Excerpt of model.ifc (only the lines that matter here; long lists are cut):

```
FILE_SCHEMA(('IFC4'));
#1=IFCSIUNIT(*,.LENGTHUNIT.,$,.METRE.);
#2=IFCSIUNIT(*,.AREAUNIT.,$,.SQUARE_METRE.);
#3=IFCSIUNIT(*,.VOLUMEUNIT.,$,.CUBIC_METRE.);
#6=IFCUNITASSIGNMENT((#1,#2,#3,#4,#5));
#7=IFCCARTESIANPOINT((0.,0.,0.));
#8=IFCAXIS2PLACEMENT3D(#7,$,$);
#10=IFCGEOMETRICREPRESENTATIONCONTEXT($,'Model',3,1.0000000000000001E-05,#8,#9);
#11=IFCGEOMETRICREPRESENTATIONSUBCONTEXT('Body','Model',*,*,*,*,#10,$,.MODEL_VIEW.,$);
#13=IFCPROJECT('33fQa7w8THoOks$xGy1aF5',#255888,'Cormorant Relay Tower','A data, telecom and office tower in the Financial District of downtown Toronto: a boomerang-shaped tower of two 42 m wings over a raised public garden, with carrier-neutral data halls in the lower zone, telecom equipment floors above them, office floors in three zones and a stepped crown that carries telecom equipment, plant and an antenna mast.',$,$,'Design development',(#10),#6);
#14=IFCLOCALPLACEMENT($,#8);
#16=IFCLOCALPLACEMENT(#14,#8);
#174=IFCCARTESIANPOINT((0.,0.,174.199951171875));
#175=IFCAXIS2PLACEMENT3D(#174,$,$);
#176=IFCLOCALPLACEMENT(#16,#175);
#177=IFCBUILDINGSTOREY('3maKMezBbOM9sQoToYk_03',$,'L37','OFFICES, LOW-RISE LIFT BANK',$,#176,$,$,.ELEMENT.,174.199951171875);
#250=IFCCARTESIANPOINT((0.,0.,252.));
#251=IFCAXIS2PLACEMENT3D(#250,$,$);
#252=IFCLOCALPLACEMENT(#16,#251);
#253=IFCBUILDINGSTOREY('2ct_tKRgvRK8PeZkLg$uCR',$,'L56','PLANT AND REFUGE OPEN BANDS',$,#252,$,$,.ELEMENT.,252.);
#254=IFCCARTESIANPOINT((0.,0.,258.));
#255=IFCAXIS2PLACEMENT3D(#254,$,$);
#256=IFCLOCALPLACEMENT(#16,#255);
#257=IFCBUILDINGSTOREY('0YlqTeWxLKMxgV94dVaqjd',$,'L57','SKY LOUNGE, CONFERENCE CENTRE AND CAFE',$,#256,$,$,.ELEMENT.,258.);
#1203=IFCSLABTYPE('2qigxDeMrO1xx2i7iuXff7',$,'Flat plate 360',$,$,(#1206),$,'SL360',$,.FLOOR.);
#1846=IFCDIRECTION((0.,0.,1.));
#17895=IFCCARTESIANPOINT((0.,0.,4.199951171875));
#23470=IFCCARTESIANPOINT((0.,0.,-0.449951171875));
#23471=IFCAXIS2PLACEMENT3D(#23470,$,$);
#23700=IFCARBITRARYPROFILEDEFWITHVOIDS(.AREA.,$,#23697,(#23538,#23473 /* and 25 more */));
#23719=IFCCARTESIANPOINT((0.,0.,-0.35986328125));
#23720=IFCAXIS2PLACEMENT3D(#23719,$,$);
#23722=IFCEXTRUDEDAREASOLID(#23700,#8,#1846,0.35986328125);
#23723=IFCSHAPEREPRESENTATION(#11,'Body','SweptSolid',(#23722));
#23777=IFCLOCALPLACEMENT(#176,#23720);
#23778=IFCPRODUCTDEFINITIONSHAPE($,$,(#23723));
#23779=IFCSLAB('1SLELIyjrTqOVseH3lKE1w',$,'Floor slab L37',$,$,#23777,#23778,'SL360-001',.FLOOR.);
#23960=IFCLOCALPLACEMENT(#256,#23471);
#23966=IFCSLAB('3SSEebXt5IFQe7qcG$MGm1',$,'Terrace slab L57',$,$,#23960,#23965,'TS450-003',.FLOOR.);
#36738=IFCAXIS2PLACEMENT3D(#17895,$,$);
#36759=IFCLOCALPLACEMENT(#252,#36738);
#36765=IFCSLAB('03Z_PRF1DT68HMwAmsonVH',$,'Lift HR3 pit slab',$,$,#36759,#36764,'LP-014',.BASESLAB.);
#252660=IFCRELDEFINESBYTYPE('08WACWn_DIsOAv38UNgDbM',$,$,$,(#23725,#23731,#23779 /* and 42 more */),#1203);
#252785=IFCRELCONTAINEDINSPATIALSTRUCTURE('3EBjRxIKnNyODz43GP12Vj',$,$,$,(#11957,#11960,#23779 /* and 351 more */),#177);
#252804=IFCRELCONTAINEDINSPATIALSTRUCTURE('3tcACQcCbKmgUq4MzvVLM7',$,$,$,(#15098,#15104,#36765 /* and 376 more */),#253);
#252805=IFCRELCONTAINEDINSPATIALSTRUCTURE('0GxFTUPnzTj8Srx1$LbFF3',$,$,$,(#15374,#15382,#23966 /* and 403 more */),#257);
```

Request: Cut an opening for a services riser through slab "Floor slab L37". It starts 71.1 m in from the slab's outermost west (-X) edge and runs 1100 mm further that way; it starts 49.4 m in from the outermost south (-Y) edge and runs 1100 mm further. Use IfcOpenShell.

```python
import numpy as np
import ifcopenshell
import ifcopenshell.api.feature
import ifcopenshell.api.geometry
import ifcopenshell.api.root
import ifcopenshell.geom
import ifcopenshell.util.placement
import ifcopenshell.util.representation
import ifcopenshell.util.shape
import ifcopenshell.util.unit

model = ifcopenshell.open("model.ifc")
unit_scale = ifcopenshell.util.unit.calculate_unit_scale(model)
settings = ifcopenshell.geom.settings()


def volume(element):
    """Net volume in cubic metres, openings subtracted."""
    shape = ifcopenshell.geom.create_shape(settings, element)
    return ifcopenshell.util.shape.get_volume(shape.geometry)


slab = model.by_guid("1SLELIyjrTqOVseH3lKE1w")
before = volume(slab)

# Extent in the slab's own axes, in metres. The edges named are its -X and -Y sides.
slab_shape = ifcopenshell.geom.create_shape(settings, slab)
vertices = ifcopenshell.util.shape.get_vertices(slab_shape.geometry)
x_min, y_min, bottom = vertices.min(axis=0)
top = vertices[:, 2].max()

opening = ifcopenshell.api.root.create_entity(model, ifc_class="IfcOpeningElement", name="Services riser opening", predefined_type="OPENING")
context = ifcopenshell.util.representation.get_context(model, "Model", "Body", "MODEL_VIEW")
width, depth = 1.1, 1.1
outline = [(0.0, 0.0), (width, 0.0), (width, depth), (0.0, depth), (0.0, 0.0)]
# Overshoot both faces by 50 mm so the cut is clean.
shape = ifcopenshell.api.geometry.add_slab_representation(
    model, context=context, depth=top - bottom + 0.1, polyline=outline
)
ifcopenshell.api.geometry.assign_representation(model, product=opening, representation=shape)

matrix = ifcopenshell.util.placement.get_local_placement(slab.ObjectPlacement)
matrix[:, 3] = matrix @ np.append(np.array([x_min + 71.1, y_min + 49.4, bottom - 0.05]) / unit_scale, 1.0)
ifcopenshell.api.geometry.edit_object_placement(model, product=opening, matrix=matrix, is_si=False)
ifcopenshell.api.feature.add_feature(model, feature=opening, element=slab)

after = volume(slab)

print(f"slab volume {before:.3f} -> {after:.3f} m3")

model.write("model_edited.ifc")
```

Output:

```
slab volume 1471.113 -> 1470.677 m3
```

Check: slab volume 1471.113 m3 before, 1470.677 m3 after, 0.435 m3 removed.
